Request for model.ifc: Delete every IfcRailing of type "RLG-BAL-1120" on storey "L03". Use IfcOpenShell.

First a look at what the model holds.

```python
import ifcopenshell
import ifcopenshell.util.element

model = ifcopenshell.open("model.ifc")
print(model.schema)
storey = next(s for s in model.by_type("IfcBuildingStorey") if s.Name == "L03")
railings = [e for e in ifcopenshell.util.element.get_decomposition(storey) if e.is_a("IfcRailing")]
seen = {}
for e in railings:
    element_type = ifcopenshell.util.element.get_type(e)
    name = element_type.Name if element_type not in (None, e) else None
    seen[name] = seen.get(name, 0) + 1
for name, count in sorted(seen.items(), key=str):
    print(count, "x", name)
```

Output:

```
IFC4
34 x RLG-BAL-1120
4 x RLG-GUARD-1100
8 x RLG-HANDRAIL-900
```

```python
import ifcopenshell
import ifcopenshell.api.root
import ifcopenshell.util.element

model = ifcopenshell.open("model.ifc")

storey = next(s for s in model.by_type("IfcBuildingStorey") if s.Name == "L03")
railings = [e for e in ifcopenshell.util.element.get_decomposition(storey) if e.is_a("IfcRailing")]
targets = [e for e in railings if (t := ifcopenshell.util.element.get_type(e)) not in (None, e) and t.Name == "RLG-BAL-1120"]

for e in targets:
    ifcopenshell.api.root.remove_product(model, product=e)
print(len(targets), "removed")

model.write("model_rev.ifc")
```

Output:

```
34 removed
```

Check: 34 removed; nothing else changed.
